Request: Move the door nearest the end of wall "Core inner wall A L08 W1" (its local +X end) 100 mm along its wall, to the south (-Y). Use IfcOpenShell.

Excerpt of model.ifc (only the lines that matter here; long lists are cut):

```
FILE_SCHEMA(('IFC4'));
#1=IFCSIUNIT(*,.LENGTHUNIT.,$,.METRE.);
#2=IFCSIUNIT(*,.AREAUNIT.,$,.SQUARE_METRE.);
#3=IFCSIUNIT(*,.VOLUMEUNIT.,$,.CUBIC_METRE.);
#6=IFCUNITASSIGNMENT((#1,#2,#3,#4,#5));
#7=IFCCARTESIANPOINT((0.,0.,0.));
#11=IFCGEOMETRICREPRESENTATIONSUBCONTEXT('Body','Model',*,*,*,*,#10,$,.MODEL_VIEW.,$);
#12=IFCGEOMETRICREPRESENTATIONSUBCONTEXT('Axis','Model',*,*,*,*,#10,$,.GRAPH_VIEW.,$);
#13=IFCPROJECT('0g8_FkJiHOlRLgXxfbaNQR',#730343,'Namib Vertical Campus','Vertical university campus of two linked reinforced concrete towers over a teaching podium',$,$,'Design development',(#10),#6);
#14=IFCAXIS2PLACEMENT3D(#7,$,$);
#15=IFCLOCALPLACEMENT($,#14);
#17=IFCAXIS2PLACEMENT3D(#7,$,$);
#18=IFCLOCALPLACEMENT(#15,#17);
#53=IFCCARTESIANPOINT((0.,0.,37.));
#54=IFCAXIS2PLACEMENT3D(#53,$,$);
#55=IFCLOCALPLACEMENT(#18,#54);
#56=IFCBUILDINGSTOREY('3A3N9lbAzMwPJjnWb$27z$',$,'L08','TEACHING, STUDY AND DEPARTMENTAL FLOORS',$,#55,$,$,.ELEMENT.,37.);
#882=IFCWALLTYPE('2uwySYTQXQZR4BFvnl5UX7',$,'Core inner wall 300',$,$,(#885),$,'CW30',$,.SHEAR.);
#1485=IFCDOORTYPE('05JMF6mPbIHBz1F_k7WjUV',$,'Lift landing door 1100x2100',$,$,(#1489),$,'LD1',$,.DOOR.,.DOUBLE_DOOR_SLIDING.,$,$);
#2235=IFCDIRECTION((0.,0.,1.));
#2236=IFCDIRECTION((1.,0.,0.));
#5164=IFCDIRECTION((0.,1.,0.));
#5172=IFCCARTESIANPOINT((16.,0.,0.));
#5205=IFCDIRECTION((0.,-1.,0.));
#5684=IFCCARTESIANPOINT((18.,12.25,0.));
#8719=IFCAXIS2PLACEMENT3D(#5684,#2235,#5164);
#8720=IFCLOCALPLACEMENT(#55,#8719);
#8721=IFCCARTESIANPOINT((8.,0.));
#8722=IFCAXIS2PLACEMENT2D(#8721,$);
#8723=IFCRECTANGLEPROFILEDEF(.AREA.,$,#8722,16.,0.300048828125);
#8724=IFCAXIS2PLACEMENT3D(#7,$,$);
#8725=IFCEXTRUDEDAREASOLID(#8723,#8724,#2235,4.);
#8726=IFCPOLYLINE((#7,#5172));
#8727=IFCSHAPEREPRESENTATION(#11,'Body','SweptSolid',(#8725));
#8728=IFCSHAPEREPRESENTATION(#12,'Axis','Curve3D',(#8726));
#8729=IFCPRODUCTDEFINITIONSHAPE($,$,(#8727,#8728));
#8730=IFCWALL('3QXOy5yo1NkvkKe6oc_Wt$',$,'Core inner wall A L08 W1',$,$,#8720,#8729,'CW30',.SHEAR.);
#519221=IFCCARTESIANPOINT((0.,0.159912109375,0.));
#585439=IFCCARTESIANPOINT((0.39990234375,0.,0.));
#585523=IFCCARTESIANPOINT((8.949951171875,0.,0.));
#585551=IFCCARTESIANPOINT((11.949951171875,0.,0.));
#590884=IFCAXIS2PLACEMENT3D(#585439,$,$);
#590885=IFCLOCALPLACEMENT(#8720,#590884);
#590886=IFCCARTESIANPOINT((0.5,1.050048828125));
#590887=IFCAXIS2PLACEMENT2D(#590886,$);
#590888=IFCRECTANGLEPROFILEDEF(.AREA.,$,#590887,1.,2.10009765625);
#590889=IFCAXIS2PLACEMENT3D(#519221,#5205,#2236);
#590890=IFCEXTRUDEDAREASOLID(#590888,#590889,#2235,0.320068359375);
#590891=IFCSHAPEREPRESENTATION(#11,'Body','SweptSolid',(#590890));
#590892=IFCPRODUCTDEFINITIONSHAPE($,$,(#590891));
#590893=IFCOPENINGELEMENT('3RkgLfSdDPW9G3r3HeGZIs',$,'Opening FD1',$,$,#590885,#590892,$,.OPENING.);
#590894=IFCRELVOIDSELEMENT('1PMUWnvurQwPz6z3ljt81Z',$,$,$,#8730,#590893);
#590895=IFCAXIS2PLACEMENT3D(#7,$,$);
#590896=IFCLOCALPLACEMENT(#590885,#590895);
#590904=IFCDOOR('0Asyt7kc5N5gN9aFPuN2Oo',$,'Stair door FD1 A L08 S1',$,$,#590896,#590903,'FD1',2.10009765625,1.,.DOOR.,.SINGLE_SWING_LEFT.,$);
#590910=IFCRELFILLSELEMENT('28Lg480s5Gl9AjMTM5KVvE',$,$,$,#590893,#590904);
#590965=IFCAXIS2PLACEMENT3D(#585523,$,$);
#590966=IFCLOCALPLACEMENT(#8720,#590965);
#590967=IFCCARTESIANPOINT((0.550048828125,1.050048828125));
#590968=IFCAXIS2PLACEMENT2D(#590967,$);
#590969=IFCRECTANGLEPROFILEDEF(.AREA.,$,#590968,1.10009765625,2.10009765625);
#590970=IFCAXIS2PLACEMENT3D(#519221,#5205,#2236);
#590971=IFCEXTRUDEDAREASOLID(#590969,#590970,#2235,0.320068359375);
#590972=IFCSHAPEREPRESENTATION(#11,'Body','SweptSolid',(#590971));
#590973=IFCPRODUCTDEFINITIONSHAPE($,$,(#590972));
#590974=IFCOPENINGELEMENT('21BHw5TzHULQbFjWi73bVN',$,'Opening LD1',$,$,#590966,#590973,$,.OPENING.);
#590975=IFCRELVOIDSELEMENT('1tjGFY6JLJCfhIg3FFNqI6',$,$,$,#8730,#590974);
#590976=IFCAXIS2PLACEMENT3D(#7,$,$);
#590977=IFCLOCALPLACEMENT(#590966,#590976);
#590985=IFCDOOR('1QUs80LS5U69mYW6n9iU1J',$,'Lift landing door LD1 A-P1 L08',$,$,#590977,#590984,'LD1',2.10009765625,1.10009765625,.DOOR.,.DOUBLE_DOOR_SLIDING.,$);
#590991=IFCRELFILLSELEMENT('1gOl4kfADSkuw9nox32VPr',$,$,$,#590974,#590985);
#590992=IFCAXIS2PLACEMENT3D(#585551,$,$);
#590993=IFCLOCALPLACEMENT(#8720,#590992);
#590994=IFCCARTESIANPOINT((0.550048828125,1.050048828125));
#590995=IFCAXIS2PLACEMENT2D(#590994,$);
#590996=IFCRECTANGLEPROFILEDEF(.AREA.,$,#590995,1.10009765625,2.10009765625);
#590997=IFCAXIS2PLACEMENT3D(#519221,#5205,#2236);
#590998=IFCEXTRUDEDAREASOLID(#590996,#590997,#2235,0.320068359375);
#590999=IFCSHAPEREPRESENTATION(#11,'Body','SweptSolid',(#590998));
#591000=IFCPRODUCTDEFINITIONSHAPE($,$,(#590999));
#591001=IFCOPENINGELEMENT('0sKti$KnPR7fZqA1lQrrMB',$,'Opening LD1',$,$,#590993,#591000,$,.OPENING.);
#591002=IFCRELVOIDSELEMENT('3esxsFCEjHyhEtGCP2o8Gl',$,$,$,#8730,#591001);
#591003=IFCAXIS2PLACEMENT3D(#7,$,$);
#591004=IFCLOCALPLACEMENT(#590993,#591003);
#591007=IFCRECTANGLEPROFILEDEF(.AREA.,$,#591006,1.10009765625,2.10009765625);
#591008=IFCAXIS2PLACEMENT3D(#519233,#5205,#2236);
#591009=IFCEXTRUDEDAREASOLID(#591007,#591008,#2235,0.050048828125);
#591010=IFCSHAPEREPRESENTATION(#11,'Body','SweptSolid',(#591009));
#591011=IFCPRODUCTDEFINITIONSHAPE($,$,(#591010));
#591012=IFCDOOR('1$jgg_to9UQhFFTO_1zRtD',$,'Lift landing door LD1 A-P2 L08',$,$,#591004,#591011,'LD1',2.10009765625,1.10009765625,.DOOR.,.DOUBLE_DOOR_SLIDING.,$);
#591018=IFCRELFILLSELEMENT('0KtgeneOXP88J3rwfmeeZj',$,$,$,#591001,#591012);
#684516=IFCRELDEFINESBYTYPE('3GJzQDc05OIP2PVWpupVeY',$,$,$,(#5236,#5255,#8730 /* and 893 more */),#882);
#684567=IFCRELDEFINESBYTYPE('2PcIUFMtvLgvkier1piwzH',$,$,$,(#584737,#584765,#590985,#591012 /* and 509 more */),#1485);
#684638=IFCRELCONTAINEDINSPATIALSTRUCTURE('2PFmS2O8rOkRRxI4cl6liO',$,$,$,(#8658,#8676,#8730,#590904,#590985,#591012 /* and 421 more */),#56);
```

```python
import ifcopenshell
import ifcopenshell.api.geometry
import ifcopenshell.util.placement

model = ifcopenshell.open("model.ifc")

door = model.by_id(591012)
opening = door.FillsVoids[0].RelatingOpeningElement
wall = opening.VoidsElements[0].RelatingBuildingElement

wall_matrix = ifcopenshell.util.placement.get_local_placement(wall.ObjectPlacement)
shift = wall_matrix[:3, 0] * -0.1
before = ifcopenshell.util.placement.get_local_placement(door.ObjectPlacement)[:3, 3].copy()

# The door is placed relative to its opening, so it follows when the opening moves.
matrix = ifcopenshell.util.placement.get_local_placement(opening.ObjectPlacement)
matrix[:3, 3] += shift
ifcopenshell.api.geometry.edit_object_placement(
    model, product=opening, matrix=matrix, is_si=False, should_transform_children=True
)

after = ifcopenshell.util.placement.get_local_placement(door.ObjectPlacement)[:3, 3]
print("door moved by", (after - before).round(3) + 0.0)

model.write("model_updated.ifc")
```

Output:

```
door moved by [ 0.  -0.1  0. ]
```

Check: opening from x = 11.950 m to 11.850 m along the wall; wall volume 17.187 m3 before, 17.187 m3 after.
